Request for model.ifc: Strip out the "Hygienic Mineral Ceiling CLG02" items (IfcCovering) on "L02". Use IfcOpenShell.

First a look at what the model holds.

```python
import ifcopenshell
import ifcopenshell.util.element

model = ifcopenshell.open("model.ifc")
print(model.schema)
storey = next(s for s in model.by_type("IfcBuildingStorey") if s.Name == "L02")
coverings = [e for e in ifcopenshell.util.element.get_decomposition(storey) if e.is_a("IfcCovering")]
seen = {}
for e in coverings:
    element_type = ifcopenshell.util.element.get_type(e)
    name = element_type.Name if element_type not in (None, e) else None
    seen[name] = seen.get(name, 0) + 1
for name, count in sorted(seen.items(), key=str):
    print(count, "x", name)
```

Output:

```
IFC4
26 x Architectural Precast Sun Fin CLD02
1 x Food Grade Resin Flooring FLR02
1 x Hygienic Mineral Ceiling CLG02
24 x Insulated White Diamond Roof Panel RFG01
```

```python
import ifcopenshell
import ifcopenshell.api.root
import ifcopenshell.util.element

model = ifcopenshell.open("model.ifc")

storey = next(s for s in model.by_type("IfcBuildingStorey") if s.Name == "L02")
coverings = [e for e in ifcopenshell.util.element.get_decomposition(storey) if e.is_a("IfcCovering")]
targets = [e for e in coverings if (t := ifcopenshell.util.element.get_type(e)) not in (None, e) and t.Name == "Hygienic Mineral Ceiling CLG02"]

for e in targets:
    ifcopenshell.api.root.remove_product(model, product=e)
print(len(targets), "removed")

model.write("model_updated.ifc")
```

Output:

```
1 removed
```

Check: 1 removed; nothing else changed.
